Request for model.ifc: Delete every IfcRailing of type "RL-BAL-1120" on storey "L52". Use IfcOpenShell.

First a look at what the model holds.

```python
import ifcopenshell
import ifcopenshell.util.element

model = ifcopenshell.open("model.ifc")
print(model.schema)
storey = next(s for s in model.by_type("IfcBuildingStorey") if s.Name == "L52")
railings = [e for e in ifcopenshell.util.element.get_decomposition(storey) if e.is_a("IfcRailing")]
seen = {}
for e in railings:
    element_type = ifcopenshell.util.element.get_type(e)
    name = element_type.Name if element_type not in (None, e) else None
    seen[name] = seen.get(name, 0) + 1
for name, count in sorted(seen.items(), key=str):
    print(count, "x", name)
```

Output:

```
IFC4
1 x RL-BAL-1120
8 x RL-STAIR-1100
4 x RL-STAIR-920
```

```python
import ifcopenshell
import ifcopenshell.api.root
import ifcopenshell.util.element

model = ifcopenshell.open("model.ifc")

storey = next(s for s in model.by_type("IfcBuildingStorey") if s.Name == "L52")
railings = [e for e in ifcopenshell.util.element.get_decomposition(storey) if e.is_a("IfcRailing")]
targets = [e for e in railings if (t := ifcopenshell.util.element.get_type(e)) not in (None, e) and t.Name == "RL-BAL-1120"]

for e in targets:
    ifcopenshell.api.root.remove_product(model, product=e)
print(len(targets), "removed")

model.write("model_rev.ifc")
```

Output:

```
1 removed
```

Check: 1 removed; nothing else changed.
